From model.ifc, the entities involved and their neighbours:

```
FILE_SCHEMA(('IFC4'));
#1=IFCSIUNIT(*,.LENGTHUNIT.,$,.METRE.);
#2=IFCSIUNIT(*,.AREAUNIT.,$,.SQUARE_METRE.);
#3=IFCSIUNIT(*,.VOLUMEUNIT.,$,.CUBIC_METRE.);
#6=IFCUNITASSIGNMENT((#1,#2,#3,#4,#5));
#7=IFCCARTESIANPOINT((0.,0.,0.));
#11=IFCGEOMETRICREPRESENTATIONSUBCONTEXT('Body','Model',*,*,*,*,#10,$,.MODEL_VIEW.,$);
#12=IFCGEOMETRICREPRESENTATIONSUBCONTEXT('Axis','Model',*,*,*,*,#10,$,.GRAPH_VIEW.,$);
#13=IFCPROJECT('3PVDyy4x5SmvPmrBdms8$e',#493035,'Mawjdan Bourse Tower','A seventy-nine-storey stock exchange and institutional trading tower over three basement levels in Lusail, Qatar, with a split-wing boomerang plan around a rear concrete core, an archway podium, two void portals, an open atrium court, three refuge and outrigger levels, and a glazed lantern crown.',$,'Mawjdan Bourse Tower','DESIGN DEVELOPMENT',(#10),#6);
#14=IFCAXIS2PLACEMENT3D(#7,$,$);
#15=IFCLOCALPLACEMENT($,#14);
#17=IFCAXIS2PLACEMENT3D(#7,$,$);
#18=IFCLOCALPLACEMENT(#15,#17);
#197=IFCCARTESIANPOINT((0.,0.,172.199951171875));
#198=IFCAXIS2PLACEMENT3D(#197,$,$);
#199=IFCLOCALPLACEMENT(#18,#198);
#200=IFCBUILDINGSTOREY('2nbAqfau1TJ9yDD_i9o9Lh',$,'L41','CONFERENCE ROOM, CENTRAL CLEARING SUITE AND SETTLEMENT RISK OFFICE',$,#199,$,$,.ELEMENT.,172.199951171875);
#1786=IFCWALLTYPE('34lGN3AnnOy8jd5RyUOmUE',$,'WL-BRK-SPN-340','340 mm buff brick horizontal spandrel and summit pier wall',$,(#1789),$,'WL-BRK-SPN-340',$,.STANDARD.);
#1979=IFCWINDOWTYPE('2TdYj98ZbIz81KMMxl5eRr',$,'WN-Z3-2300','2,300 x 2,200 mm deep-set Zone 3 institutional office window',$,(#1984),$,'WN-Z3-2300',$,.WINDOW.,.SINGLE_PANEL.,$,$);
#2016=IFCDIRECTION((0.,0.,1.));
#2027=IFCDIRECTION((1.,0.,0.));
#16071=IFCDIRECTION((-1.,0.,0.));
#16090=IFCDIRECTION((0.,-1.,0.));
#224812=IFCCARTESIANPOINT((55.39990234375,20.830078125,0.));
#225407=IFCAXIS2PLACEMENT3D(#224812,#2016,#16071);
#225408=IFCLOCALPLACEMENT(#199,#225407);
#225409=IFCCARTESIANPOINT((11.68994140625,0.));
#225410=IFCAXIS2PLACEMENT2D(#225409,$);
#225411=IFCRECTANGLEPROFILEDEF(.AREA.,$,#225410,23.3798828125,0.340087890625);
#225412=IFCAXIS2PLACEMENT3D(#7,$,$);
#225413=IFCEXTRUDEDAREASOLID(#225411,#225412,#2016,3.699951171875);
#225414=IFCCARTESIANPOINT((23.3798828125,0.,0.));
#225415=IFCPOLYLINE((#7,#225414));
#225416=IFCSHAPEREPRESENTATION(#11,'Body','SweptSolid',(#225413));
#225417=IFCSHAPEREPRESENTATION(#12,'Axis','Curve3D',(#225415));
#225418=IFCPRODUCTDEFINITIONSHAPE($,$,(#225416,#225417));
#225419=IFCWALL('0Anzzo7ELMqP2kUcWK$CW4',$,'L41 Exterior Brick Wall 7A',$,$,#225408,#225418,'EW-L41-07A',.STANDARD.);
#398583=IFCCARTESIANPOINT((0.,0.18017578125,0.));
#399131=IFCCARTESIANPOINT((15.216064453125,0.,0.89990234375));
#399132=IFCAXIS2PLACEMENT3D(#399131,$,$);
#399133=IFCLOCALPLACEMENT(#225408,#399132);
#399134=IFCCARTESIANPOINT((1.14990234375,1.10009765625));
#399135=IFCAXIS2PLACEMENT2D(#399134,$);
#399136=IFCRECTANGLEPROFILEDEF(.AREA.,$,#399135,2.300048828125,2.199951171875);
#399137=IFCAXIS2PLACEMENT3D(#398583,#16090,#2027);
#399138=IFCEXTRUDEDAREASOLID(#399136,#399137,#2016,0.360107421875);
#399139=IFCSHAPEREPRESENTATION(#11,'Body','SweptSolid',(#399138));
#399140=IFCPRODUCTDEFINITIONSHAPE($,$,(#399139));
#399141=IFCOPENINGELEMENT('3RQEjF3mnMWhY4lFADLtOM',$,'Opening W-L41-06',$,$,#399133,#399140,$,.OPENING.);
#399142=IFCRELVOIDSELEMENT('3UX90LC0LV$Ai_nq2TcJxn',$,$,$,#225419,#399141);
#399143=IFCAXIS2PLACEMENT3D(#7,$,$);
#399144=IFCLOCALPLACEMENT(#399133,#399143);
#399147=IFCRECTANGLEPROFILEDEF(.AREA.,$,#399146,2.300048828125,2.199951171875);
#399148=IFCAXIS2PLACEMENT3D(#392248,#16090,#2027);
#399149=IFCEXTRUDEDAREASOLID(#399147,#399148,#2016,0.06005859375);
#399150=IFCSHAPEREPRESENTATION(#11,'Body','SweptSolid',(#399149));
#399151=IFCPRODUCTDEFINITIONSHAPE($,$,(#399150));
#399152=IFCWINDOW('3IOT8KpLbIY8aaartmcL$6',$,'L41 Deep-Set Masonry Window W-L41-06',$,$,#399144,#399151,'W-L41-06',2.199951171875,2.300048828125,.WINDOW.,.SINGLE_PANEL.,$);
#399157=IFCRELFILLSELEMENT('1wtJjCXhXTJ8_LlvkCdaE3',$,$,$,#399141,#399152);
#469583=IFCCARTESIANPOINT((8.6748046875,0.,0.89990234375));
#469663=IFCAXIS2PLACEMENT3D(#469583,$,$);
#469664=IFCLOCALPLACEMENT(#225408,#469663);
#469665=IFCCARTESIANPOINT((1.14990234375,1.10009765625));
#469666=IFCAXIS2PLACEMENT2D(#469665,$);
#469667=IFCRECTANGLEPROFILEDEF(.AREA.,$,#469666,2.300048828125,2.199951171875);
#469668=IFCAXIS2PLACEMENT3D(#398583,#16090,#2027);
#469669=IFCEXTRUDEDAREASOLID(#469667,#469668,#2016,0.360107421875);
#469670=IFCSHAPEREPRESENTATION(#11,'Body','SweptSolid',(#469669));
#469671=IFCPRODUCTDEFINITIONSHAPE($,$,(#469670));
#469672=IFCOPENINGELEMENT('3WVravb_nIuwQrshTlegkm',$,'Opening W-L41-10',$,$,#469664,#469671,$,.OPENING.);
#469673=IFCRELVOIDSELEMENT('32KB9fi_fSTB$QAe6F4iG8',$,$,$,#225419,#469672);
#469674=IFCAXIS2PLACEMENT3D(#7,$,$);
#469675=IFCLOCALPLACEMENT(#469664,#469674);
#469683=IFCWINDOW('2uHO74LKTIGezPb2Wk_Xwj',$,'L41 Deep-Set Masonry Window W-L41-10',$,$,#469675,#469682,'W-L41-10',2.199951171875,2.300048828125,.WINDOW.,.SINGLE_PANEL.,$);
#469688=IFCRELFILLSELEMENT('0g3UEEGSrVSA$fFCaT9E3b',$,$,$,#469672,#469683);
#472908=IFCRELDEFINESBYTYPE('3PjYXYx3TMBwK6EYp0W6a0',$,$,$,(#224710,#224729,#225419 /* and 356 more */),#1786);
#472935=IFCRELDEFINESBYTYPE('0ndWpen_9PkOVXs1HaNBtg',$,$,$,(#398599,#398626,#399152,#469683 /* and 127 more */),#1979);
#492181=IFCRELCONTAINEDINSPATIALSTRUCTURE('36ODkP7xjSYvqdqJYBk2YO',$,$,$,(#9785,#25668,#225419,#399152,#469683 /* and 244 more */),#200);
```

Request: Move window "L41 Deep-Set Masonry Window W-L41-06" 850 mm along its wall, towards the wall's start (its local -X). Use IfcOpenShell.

```python
import ifcopenshell
import ifcopenshell.api.geometry
import ifcopenshell.util.placement

model = ifcopenshell.open("model.ifc")

window = model.by_guid("3IOT8KpLbIY8aaartmcL$6")
opening = window.FillsVoids[0].RelatingOpeningElement
wall = opening.VoidsElements[0].RelatingBuildingElement

wall_matrix = ifcopenshell.util.placement.get_local_placement(wall.ObjectPlacement)
shift = wall_matrix[:3, 0] * -0.85
before = ifcopenshell.util.placement.get_local_placement(window.ObjectPlacement)[:3, 3].copy()

# The window is placed relative to its opening, so it follows when the opening moves.
matrix = ifcopenshell.util.placement.get_local_placement(opening.ObjectPlacement)
matrix[:3, 3] += shift
ifcopenshell.api.geometry.edit_object_placement(
    model, product=opening, matrix=matrix, is_si=False, should_transform_children=True
)

after = ifcopenshell.util.placement.get_local_placement(window.ObjectPlacement)[:3, 3]
print("window moved by", (after - before).round(3) + 0.0)

model.write("model_rev.ifc")
```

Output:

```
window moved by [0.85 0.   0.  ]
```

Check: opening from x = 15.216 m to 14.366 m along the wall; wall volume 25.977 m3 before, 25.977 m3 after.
